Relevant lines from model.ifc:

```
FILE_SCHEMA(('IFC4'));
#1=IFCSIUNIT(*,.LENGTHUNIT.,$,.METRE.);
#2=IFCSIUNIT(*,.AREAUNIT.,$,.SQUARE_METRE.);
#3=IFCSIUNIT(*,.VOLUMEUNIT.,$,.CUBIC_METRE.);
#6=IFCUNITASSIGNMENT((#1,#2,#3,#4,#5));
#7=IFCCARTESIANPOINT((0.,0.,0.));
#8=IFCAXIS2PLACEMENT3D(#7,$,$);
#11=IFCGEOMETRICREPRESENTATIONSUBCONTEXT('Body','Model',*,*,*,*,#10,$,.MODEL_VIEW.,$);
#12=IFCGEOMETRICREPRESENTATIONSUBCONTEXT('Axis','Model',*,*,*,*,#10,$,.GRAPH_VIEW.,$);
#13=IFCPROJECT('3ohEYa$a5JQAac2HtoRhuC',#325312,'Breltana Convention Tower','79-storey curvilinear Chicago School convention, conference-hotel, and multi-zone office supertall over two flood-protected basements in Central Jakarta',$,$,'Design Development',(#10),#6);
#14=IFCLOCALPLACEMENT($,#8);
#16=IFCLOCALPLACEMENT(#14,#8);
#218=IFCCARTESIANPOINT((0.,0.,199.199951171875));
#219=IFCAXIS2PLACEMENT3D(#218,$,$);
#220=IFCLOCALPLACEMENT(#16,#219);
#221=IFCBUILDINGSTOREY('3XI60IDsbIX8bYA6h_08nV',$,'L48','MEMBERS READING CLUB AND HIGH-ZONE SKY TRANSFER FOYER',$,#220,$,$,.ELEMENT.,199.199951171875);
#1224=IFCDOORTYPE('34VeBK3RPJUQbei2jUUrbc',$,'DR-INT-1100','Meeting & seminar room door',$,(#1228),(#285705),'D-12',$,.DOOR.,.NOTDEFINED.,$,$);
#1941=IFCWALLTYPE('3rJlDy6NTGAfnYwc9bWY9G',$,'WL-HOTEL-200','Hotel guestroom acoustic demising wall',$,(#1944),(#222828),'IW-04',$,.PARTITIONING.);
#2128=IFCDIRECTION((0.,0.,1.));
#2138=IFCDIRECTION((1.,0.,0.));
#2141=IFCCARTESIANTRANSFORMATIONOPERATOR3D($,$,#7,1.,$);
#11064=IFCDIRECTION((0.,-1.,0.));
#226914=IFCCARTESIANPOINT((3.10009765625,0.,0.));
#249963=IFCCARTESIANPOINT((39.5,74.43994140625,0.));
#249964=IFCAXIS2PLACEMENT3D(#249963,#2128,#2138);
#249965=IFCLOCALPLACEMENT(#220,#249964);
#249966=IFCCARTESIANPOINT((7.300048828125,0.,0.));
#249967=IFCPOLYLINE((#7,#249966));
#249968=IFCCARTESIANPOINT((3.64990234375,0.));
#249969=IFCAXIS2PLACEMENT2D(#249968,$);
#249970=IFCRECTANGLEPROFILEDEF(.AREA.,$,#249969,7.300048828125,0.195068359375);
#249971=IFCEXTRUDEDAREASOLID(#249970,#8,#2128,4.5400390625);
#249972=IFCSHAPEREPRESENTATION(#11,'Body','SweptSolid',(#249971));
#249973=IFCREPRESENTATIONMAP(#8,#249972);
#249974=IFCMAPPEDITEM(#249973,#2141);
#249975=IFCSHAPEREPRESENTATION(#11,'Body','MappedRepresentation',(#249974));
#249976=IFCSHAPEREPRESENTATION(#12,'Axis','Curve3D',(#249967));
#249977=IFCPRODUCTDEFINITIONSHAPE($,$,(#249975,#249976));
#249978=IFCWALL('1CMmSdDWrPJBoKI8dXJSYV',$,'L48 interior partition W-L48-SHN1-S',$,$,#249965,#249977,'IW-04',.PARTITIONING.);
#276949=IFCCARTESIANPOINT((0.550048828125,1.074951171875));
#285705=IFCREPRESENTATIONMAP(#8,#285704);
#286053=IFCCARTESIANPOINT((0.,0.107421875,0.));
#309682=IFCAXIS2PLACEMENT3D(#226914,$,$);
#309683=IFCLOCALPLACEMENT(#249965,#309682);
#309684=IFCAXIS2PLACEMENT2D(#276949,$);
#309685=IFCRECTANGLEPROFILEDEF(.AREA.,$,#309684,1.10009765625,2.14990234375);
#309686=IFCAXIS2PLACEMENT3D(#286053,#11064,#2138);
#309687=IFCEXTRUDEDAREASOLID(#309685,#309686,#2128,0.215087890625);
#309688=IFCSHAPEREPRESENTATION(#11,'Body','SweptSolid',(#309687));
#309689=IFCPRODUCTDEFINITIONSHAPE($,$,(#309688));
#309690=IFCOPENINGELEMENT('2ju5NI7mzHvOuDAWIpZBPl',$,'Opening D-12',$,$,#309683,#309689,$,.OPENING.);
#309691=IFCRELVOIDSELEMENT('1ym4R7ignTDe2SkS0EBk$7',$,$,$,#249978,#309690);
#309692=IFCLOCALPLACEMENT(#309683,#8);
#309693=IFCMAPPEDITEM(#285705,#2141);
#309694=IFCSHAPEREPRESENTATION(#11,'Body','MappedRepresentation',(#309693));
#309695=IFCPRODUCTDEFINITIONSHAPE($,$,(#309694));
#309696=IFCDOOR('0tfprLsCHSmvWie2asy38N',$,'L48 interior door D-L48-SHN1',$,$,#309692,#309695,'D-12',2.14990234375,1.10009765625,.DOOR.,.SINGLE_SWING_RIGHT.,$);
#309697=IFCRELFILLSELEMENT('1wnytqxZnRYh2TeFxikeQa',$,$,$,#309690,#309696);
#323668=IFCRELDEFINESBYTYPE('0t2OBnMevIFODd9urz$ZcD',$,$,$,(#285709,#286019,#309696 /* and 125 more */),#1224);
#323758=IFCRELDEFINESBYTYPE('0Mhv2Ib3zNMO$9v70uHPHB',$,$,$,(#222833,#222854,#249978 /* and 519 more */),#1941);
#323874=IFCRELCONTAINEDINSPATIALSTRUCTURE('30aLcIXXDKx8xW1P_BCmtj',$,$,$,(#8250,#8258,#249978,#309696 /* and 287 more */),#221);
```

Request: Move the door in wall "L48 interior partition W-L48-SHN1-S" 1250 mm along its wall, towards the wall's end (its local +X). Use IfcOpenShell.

```python
import ifcopenshell
import ifcopenshell.api.geometry
import ifcopenshell.util.placement
import ifcopenshell.util.unit

model = ifcopenshell.open("model.ifc")
unit_scale = ifcopenshell.util.unit.calculate_unit_scale(model)

door = model.by_guid("0tfprLsCHSmvWie2asy38N")
opening = door.FillsVoids[0].RelatingOpeningElement
wall = opening.VoidsElements[0].RelatingBuildingElement

wall_matrix = ifcopenshell.util.placement.get_local_placement(wall.ObjectPlacement)
shift = wall_matrix[:3, 0] * 1.25 / unit_scale
before = ifcopenshell.util.placement.get_local_placement(door.ObjectPlacement)[:3, 3].copy()

# The door is placed relative to its opening, so it follows when the opening moves.
matrix = ifcopenshell.util.placement.get_local_placement(opening.ObjectPlacement)
matrix[:3, 3] += shift
ifcopenshell.api.geometry.edit_object_placement(
    model, product=opening, matrix=matrix, is_si=False, should_transform_children=True
)

after = ifcopenshell.util.placement.get_local_placement(door.ObjectPlacement)[:3, 3]
print("door moved by", (after - before).round(3) + 0.0)

model.write("model-out.ifc")
```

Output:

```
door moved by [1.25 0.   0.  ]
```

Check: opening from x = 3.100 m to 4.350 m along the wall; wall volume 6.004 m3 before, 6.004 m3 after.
